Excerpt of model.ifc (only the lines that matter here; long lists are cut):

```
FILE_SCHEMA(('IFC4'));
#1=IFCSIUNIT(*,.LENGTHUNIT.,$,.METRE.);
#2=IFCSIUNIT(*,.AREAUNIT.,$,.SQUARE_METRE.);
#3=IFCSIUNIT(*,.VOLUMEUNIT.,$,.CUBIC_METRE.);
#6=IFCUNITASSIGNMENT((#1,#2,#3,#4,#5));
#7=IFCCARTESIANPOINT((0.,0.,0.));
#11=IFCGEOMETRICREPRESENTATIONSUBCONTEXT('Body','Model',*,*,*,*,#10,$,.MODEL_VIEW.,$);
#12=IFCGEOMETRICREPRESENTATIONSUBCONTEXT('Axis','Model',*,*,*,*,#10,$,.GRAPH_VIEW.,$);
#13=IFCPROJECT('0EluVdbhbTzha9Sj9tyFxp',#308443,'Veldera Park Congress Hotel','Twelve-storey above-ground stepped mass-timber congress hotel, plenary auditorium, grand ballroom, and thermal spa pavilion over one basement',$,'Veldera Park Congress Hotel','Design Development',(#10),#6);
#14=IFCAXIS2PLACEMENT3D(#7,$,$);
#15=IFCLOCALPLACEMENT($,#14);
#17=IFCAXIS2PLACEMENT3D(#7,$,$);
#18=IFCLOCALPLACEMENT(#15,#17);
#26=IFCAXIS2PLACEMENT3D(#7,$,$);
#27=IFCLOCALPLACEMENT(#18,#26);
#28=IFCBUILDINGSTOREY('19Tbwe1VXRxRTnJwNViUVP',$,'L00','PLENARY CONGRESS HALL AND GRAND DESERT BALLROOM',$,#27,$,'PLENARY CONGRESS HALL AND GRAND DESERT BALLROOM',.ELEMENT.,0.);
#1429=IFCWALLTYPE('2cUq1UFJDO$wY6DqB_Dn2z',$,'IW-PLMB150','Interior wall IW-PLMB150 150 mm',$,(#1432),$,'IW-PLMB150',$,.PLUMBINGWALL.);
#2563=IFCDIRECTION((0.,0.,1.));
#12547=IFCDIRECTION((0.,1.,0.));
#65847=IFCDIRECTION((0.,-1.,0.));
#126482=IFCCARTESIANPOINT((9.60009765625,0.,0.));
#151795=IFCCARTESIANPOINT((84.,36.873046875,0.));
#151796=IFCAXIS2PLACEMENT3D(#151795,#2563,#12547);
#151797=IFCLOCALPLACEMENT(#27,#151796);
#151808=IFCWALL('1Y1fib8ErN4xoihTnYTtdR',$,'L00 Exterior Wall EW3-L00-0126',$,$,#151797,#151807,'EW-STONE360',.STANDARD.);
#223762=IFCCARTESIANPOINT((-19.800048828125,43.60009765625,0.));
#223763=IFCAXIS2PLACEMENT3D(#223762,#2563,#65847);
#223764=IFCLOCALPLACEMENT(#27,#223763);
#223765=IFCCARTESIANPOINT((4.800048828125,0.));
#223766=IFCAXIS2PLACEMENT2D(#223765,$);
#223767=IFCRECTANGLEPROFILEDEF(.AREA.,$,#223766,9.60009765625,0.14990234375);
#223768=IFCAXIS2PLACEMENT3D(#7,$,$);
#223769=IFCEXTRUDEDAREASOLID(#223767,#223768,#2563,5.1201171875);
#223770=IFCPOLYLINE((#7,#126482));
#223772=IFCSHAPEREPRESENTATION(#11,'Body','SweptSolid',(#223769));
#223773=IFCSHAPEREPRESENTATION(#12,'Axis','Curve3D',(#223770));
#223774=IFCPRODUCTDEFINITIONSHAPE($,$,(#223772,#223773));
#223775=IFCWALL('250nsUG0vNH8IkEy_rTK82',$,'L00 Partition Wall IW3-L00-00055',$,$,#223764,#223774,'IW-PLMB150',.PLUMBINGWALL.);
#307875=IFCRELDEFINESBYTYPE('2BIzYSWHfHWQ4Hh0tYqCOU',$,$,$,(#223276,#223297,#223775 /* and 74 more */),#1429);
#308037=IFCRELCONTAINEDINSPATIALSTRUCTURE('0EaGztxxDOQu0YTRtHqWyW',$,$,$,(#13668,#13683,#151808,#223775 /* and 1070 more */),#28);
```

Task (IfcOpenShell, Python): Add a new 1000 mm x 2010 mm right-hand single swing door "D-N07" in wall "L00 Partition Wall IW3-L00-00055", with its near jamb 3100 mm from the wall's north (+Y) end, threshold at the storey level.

```python
import numpy as np
import ifcopenshell
import ifcopenshell.api.feature
import ifcopenshell.api.geometry
import ifcopenshell.api.root
import ifcopenshell.api.spatial
import ifcopenshell.geom
import ifcopenshell.util.element
import ifcopenshell.util.placement
import ifcopenshell.util.representation
import ifcopenshell.util.shape
import ifcopenshell.util.unit

model = ifcopenshell.open("model.ifc")
unit_scale = ifcopenshell.util.unit.calculate_unit_scale(model)
settings = ifcopenshell.geom.settings()


def volume(element):
    """Net volume in cubic metres, openings subtracted."""
    shape = ifcopenshell.geom.create_shape(settings, element)
    return ifcopenshell.util.shape.get_volume(shape.geometry)


wall = model.by_guid("250nsUG0vNH8IkEy_rTK82")
storey = ifcopenshell.util.element.get_container(wall, ifc_class="IfcBuildingStorey")
context = ifcopenshell.util.representation.get_context(model, "Model", "Body", "MODEL_VIEW")
before = volume(wall)

width, height, from_end, sill = 1, 2.01, 3.1, 0.0  # metres

# The wall runs along its own X axis, and the end named is its -X end.
wall_shape = ifcopenshell.geom.create_shape(settings, wall)
x, y, z = ifcopenshell.util.shape.get_vertices(wall_shape.geometry).T
start = x.min() + from_end
face, thickness = float(y.min()), float(y.max() - y.min())
wall_matrix = ifcopenshell.util.placement.get_local_placement(wall.ObjectPlacement)
level = ifcopenshell.util.placement.get_local_placement(storey.ObjectPlacement)[2, 3]


def in_wall(x, y):
    """Placement at x, y metres in the wall's axes, at sill height."""
    matrix = wall_matrix.copy()
    matrix[:, 3] = wall_matrix @ np.array([x / unit_scale, y / unit_scale, 0.0, 1.0])
    matrix[2, 3] = level + sill / unit_scale
    return matrix


# Opening: a box that overshoots both wall faces by 50 mm.
opening = ifcopenshell.api.root.create_entity(model, ifc_class="IfcOpeningElement", predefined_type="OPENING")
box = ifcopenshell.api.geometry.add_wall_representation(
    model, context=context, length=width, height=height, thickness=thickness + 0.1
)
ifcopenshell.api.geometry.assign_representation(model, product=opening, representation=box)
ifcopenshell.api.geometry.edit_object_placement(model, product=opening, matrix=in_wall(start, face - 0.05), is_si=False)
ifcopenshell.api.feature.add_feature(model, feature=opening, element=wall)

door = ifcopenshell.api.root.create_entity(model, ifc_class="IfcDoor", name="D-N07", predefined_type="DOOR")
door.OverallWidth, door.OverallHeight = width / unit_scale, height / unit_scale
door.OperationType = "SINGLE_SWING_RIGHT"
body = ifcopenshell.api.geometry.add_door_representation(
    model,
    context=context,
    overall_width=door.OverallWidth,
    overall_height=door.OverallHeight,
    operation_type="SINGLE_SWING_RIGHT",
    lining_properties={"LiningDepth": thickness / unit_scale, "ThresholdDepth": thickness / unit_scale},
)
ifcopenshell.api.geometry.assign_representation(model, product=door, representation=body)
ifcopenshell.api.spatial.assign_container(model, products=[door], relating_structure=storey)
ifcopenshell.api.feature.add_filling(model, opening=opening, element=door)

# The lining spans the wall, so the door starts at the wall face.
ifcopenshell.api.geometry.edit_object_placement(model, product=door, matrix=in_wall(start, face), is_si=False)

after = volume(wall)

print(f"wall volume {before:.3f} -> {after:.3f} m3")

model.write("model_edited.ifc")
```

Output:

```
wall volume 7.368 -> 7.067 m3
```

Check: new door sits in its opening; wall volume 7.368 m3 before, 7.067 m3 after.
